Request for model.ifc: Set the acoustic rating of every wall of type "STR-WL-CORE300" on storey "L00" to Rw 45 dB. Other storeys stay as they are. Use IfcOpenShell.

First a look at what the model holds.

```python
import ifcopenshell
import ifcopenshell.util.element

model = ifcopenshell.open("model.ifc")
print(model.schema)
storey = next(s for s in model.by_type("IfcBuildingStorey") if s.Name == "L00")
walls = [e for e in ifcopenshell.util.element.get_decomposition(storey) if e.is_a("IfcWall")]
seen = {}
for e in walls:
    element_type = ifcopenshell.util.element.get_type(e)
    key = (element_type.Name if element_type != e and element_type else None, ifcopenshell.util.element.get_pset(e, "Pset_WallCommon", "AcousticRating"))
    seen[key] = seen.get(key, 0) + 1
for (name, value), count in sorted(seen.items(), key=str):
    print(count, "x", name, "|", value)
```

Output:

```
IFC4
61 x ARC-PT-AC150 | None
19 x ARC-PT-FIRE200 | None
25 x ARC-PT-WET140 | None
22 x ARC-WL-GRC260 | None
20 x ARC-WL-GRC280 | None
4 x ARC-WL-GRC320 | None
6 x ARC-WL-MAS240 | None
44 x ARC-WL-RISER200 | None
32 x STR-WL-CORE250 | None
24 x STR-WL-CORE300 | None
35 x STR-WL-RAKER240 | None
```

```python
import ifcopenshell
import ifcopenshell.api.pset
import ifcopenshell.util.element

model = ifcopenshell.open("model.ifc")

storey = next(s for s in model.by_type("IfcBuildingStorey") if s.Name == "L00")
walls = [e for e in ifcopenshell.util.element.get_decomposition(storey) if e.is_a("IfcWall")]

count = 0
for e in walls:
    element_type = ifcopenshell.util.element.get_type(e)
    if element_type in (None, e) or element_type.Name != "STR-WL-CORE300":
        continue
    # add_pset returns the element's existing set when there is one.
    pset = ifcopenshell.api.pset.add_pset(model, product=e, name="Pset_WallCommon")
    ifcopenshell.api.pset.edit_pset(model, pset=pset, properties={"AcousticRating": "Rw 45 dB"})
    count += 1

print(count, "walls updated")

model.write("model-out.ifc")
```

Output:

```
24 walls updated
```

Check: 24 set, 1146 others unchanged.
